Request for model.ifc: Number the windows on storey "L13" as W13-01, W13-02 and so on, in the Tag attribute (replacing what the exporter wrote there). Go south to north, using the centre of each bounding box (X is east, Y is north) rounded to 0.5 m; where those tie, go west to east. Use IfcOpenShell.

First a look at what the model holds.

```python
import ifcopenshell
import ifcopenshell.util.element
import ifcopenshell.util.placement

model = ifcopenshell.open("model.ifc")
print(model.schema)
storey = next(s for s in model.by_type("IfcBuildingStorey") if s.Name == "L13")
windows = [e for e in ifcopenshell.util.element.get_decomposition(storey) if e.is_a("IfcWindow")]
for e in sorted(windows, key=lambda e: e.id()):
    origin = ifcopenshell.util.placement.get_local_placement(e.ObjectPlacement)[:3, 3]
    print(e.id(), e.Tag, e.Name, origin.round(2) + 0.0, sep=" | ")
```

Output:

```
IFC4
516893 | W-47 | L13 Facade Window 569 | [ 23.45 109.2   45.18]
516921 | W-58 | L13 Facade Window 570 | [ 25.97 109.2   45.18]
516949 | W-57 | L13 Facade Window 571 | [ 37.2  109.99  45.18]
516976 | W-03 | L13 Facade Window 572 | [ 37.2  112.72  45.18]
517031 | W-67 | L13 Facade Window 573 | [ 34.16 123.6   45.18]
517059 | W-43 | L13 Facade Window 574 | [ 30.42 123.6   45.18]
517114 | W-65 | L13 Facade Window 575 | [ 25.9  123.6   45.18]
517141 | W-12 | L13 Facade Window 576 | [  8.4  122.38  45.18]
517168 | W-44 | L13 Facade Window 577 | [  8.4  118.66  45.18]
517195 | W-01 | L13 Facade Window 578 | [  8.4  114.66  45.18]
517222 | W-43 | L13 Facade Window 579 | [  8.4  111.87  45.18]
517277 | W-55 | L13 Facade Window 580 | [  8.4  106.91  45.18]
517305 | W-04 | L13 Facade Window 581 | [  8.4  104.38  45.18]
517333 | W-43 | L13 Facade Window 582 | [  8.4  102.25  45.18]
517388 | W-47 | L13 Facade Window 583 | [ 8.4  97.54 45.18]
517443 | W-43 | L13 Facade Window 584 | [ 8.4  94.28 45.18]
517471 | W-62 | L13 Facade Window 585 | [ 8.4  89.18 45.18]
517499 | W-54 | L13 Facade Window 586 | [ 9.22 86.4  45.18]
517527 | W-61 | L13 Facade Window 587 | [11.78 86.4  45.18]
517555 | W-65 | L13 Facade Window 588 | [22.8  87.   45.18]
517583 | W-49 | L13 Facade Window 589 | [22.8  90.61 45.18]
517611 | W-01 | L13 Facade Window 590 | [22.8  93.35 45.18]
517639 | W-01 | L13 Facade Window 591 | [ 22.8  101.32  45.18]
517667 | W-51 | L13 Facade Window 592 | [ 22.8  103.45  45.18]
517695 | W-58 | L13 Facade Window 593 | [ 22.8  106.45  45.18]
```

```python
import ifcopenshell
import ifcopenshell.geom
import ifcopenshell.util.element
import ifcopenshell.util.shape

model = ifcopenshell.open("model.ifc")
settings = ifcopenshell.geom.settings()
settings.set("use-world-coords", True)


def centre(element):
    shape = ifcopenshell.geom.create_shape(settings, element)
    return ifcopenshell.util.shape.get_bbox_centroid(shape.geometry)


storey = next(s for s in model.by_type("IfcBuildingStorey") if s.Name == "L13")
windows = [e for e in ifcopenshell.util.element.get_decomposition(storey) if e.is_a("IfcWindow")]

# Insertion points can sit at a corner or the storey origin, so sort by the geometry (in metres).
centres = {e: centre(e) for e in windows}
windows.sort(key=lambda e: (round(centres[e][1] / 0.5), centres[e][0]))

for i, e in enumerate(windows, start=1):
    number = f"W13-{i:02d}"
    e.Tag = number
    print(e.id(), number)

model.write("model_v2.ifc")
```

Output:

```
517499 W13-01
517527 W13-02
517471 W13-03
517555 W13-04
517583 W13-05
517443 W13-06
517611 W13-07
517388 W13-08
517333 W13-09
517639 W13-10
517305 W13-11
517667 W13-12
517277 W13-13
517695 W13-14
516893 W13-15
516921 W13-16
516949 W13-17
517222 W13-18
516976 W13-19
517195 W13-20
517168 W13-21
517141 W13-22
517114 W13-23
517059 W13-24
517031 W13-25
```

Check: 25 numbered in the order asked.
